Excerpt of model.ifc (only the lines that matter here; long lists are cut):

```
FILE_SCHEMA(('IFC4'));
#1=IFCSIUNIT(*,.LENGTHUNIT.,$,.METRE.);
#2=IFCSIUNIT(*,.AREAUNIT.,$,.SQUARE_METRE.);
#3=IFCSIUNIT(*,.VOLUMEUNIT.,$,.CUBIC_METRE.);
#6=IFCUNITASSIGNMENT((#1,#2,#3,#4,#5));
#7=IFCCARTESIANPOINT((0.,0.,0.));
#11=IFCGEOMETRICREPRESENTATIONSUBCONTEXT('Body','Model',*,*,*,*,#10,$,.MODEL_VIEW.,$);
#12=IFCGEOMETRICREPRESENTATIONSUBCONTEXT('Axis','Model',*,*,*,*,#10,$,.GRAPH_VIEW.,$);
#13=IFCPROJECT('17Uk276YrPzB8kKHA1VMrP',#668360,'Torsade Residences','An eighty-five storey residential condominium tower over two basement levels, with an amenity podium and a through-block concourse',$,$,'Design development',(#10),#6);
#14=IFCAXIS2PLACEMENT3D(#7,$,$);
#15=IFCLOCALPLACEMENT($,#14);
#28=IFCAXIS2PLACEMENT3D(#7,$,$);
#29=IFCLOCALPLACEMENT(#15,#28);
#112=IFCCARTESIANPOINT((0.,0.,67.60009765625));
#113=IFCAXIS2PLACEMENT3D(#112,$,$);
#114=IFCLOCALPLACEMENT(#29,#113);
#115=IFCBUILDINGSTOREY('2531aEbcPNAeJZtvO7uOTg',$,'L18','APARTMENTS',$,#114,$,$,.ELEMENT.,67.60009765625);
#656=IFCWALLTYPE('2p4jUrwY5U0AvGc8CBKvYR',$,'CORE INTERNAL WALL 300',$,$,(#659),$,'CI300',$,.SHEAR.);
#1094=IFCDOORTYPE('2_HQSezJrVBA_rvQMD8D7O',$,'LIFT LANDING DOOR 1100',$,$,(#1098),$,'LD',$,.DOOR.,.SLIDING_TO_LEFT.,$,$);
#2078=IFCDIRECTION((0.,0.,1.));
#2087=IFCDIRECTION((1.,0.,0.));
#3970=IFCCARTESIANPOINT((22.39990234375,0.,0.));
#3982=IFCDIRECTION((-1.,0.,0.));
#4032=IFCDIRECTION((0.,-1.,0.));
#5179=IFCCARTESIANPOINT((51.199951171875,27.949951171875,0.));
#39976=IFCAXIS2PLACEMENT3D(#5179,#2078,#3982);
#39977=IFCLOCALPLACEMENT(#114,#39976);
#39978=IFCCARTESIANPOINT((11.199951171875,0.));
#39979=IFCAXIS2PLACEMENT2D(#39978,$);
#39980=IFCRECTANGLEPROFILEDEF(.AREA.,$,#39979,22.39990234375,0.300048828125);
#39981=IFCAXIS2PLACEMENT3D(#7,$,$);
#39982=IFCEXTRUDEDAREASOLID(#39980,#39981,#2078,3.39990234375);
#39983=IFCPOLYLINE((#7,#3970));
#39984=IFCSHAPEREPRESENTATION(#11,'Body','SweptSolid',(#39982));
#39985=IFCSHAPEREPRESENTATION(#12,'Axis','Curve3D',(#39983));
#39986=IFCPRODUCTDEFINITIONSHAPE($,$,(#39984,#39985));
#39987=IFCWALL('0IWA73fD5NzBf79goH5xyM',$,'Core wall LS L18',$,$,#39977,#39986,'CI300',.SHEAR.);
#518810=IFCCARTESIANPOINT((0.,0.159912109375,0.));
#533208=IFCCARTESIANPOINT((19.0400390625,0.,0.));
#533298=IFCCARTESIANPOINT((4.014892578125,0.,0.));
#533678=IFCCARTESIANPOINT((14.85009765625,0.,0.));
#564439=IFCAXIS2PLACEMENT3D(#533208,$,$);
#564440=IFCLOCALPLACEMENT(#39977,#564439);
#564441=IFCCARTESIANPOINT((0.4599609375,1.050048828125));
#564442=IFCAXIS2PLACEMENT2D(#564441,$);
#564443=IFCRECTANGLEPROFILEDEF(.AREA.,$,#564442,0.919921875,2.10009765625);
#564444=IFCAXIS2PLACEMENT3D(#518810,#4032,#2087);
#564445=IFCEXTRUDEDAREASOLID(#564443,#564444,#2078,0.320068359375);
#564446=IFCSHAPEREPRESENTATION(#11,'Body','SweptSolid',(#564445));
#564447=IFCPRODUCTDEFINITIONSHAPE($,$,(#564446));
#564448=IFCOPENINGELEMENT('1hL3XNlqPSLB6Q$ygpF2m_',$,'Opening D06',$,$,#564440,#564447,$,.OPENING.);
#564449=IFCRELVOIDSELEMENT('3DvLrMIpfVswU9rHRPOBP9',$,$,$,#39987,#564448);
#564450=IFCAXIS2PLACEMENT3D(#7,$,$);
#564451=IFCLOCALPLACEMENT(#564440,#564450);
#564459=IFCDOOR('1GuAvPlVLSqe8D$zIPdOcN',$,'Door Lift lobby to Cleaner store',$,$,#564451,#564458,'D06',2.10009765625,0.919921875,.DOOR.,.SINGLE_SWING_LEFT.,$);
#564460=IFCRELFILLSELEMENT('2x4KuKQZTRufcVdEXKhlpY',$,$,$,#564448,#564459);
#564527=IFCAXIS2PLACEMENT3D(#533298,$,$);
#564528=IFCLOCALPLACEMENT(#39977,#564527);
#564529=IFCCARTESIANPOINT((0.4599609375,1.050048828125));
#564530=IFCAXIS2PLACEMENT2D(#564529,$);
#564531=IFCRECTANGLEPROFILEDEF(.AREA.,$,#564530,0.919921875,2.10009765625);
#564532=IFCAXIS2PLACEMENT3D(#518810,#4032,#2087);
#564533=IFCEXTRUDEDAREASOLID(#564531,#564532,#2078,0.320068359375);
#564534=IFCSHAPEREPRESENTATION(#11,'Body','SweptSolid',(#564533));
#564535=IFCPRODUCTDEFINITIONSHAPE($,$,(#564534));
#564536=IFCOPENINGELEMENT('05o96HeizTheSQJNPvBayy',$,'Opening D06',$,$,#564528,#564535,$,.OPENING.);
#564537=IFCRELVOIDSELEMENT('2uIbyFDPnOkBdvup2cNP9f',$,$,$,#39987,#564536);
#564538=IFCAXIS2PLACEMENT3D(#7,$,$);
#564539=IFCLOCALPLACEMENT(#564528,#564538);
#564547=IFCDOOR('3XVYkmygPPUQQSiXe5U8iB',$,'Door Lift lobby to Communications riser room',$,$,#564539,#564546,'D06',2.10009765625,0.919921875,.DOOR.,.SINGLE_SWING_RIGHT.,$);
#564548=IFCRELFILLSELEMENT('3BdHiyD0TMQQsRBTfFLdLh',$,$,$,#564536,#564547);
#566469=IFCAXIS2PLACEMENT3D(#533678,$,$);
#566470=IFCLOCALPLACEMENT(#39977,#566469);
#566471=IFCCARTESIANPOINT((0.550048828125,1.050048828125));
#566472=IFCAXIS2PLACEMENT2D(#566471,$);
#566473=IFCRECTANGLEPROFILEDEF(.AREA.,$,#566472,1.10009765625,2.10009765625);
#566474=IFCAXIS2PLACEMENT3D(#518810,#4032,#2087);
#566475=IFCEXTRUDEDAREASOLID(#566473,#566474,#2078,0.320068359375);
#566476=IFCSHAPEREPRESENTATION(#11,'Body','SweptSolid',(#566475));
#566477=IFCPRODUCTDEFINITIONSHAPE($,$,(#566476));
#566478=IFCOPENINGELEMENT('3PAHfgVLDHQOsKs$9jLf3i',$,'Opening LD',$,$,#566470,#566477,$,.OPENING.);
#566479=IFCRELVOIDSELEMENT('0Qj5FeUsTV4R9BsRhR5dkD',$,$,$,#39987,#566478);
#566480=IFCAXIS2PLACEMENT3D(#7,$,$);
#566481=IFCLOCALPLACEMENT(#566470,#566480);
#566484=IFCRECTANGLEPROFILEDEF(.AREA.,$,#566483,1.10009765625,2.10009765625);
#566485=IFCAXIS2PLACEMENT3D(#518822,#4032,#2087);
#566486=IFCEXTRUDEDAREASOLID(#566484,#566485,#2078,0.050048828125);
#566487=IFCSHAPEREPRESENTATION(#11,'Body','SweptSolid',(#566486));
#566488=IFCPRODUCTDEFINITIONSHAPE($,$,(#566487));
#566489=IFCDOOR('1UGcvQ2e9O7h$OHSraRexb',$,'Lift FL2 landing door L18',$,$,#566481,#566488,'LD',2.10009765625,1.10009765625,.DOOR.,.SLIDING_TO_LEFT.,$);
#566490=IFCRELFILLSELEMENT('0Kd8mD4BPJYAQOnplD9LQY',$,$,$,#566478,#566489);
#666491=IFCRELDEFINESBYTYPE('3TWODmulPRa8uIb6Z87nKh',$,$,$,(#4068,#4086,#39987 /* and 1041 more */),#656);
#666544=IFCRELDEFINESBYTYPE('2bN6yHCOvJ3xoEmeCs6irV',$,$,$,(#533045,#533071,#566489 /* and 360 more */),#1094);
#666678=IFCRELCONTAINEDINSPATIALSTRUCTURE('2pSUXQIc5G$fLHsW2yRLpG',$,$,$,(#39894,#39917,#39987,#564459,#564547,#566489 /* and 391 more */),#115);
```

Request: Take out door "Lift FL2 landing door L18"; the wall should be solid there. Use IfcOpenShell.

```python
import ifcopenshell
import ifcopenshell.api.feature
import ifcopenshell.api.root
import ifcopenshell.geom
import ifcopenshell.util.shape

model = ifcopenshell.open("model.ifc")
settings = ifcopenshell.geom.settings()


def volume(element):
    """Net volume in cubic metres, openings subtracted."""
    shape = ifcopenshell.geom.create_shape(settings, element)
    return ifcopenshell.util.shape.get_volume(shape.geometry)


door = model.by_guid("1UGcvQ2e9O7h$OHSraRexb")
opening = door.FillsVoids[0].RelatingOpeningElement
wall = opening.VoidsElements[0].RelatingBuildingElement
before = volume(wall)

ifcopenshell.api.root.remove_product(model, product=door)
ifcopenshell.api.feature.remove_feature(model, feature=opening)

after = volume(wall)

print(f"wall volume {before:.3f} -> {after:.3f} m3")

model.write("model_updated.ifc")
```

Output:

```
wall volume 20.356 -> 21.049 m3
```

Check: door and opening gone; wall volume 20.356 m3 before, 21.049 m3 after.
